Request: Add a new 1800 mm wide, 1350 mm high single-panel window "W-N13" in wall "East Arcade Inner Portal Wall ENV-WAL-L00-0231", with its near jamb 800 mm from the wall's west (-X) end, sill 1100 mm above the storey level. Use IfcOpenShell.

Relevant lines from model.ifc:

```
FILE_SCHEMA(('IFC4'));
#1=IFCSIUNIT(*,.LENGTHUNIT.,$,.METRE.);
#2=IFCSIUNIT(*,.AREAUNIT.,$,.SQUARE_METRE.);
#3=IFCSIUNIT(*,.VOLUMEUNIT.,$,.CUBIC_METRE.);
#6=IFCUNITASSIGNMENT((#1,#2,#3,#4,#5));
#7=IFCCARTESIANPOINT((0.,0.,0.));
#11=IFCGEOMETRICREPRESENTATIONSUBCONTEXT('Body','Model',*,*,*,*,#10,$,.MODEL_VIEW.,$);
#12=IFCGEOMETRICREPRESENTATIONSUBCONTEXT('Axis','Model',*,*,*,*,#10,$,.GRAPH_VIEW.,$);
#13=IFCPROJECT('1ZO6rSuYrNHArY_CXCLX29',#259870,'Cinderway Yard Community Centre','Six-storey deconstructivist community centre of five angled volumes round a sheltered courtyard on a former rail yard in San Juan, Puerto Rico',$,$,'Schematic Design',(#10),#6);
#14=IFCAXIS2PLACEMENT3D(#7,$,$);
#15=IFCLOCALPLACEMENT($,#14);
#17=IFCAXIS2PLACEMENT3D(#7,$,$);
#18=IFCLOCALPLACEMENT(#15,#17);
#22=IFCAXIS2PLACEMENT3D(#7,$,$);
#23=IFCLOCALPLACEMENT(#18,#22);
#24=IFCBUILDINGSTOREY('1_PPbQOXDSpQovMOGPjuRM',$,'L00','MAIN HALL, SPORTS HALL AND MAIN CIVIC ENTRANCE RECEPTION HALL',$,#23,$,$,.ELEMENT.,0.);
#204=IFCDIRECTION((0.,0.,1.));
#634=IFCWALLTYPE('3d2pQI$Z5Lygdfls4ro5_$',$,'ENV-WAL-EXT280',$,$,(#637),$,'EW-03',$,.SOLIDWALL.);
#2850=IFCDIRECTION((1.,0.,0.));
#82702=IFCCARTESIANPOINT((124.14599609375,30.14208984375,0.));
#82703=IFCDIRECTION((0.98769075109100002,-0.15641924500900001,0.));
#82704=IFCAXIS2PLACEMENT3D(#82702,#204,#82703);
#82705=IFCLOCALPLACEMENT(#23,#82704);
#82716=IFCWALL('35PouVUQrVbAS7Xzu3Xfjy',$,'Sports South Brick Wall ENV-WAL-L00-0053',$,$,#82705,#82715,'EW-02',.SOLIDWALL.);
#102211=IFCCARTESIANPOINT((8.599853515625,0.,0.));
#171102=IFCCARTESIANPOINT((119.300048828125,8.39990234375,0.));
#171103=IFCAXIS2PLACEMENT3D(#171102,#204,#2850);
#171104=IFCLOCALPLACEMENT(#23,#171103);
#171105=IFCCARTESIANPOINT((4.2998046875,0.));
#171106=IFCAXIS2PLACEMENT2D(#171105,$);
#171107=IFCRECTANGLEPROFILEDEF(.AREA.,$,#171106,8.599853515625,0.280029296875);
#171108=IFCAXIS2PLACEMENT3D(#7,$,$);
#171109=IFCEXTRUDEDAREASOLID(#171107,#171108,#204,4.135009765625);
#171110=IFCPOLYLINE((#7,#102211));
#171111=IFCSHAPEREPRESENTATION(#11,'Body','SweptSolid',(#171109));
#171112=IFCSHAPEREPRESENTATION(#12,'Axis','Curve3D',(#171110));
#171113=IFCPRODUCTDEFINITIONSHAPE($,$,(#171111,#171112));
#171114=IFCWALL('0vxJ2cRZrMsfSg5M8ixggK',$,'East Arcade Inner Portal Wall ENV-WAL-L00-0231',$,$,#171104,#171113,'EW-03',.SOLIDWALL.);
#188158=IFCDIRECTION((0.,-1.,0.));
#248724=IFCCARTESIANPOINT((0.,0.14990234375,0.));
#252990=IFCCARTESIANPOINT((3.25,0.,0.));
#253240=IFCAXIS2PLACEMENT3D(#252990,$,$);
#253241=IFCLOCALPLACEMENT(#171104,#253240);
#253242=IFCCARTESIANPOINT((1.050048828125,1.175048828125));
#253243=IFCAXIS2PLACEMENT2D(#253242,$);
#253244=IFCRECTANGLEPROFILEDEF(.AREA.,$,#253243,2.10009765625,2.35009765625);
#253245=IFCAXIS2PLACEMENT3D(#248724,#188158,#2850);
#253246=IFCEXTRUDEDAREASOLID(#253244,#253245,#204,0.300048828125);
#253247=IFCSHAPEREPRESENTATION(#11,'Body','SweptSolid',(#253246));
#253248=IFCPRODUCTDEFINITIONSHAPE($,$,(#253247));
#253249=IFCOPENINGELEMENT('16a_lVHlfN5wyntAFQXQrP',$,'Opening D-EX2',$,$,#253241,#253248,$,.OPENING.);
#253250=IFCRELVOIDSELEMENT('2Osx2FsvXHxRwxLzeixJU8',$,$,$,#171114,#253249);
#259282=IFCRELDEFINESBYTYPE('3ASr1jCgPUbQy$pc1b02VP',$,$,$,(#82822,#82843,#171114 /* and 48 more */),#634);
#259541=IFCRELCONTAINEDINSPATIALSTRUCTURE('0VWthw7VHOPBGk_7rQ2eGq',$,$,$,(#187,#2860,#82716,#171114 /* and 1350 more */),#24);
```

```python
import numpy as np
import ifcopenshell
import ifcopenshell.api.feature
import ifcopenshell.api.geometry
import ifcopenshell.api.root
import ifcopenshell.api.spatial
import ifcopenshell.geom
import ifcopenshell.util.element
import ifcopenshell.util.placement
import ifcopenshell.util.representation
import ifcopenshell.util.shape
import ifcopenshell.util.unit

model = ifcopenshell.open("model.ifc")
unit_scale = ifcopenshell.util.unit.calculate_unit_scale(model)
settings = ifcopenshell.geom.settings()


def volume(element):
    """Net volume in cubic metres, openings subtracted."""
    shape = ifcopenshell.geom.create_shape(settings, element)
    return ifcopenshell.util.shape.get_volume(shape.geometry)


wall = model.by_guid("0vxJ2cRZrMsfSg5M8ixggK")
storey = ifcopenshell.util.element.get_container(wall, ifc_class="IfcBuildingStorey")
context = ifcopenshell.util.representation.get_context(model, "Model", "Body", "MODEL_VIEW")
before = volume(wall)

width, height, from_end, sill = 1.8, 1.35, 0.8, 1.1  # metres

# The wall runs along its own X axis, and the end named is its -X end.
wall_shape = ifcopenshell.geom.create_shape(settings, wall)
x, y, z = ifcopenshell.util.shape.get_vertices(wall_shape.geometry).T
start = x.min() + from_end
face, thickness = float(y.min()), float(y.max() - y.min())
wall_matrix = ifcopenshell.util.placement.get_local_placement(wall.ObjectPlacement)
level = ifcopenshell.util.placement.get_local_placement(storey.ObjectPlacement)[2, 3]


def in_wall(x, y):
    """Placement at x, y metres in the wall's axes, at sill height."""
    matrix = wall_matrix.copy()
    matrix[:, 3] = wall_matrix @ np.array([x / unit_scale, y / unit_scale, 0.0, 1.0])
    matrix[2, 3] = level + sill / unit_scale
    return matrix


# Opening: a box that overshoots both wall faces by 50 mm.
opening = ifcopenshell.api.root.create_entity(model, ifc_class="IfcOpeningElement", predefined_type="OPENING")
box = ifcopenshell.api.geometry.add_wall_representation(
    model, context=context, length=width, height=height, thickness=thickness + 0.1
)
ifcopenshell.api.geometry.assign_representation(model, product=opening, representation=box)
ifcopenshell.api.geometry.edit_object_placement(model, product=opening, matrix=in_wall(start, face - 0.05), is_si=False)
ifcopenshell.api.feature.add_feature(model, feature=opening, element=wall)

window = ifcopenshell.api.root.create_entity(model, ifc_class="IfcWindow", name="W-N13", predefined_type="WINDOW")
window.OverallWidth, window.OverallHeight = width / unit_scale, height / unit_scale
window.PartitioningType = "SINGLE_PANEL"
body = ifcopenshell.api.geometry.add_window_representation(
    model,
    context=context,
    overall_width=window.OverallWidth,
    overall_height=window.OverallHeight,
    partition_type="SINGLE_PANEL",
)
ifcopenshell.api.geometry.assign_representation(model, product=window, representation=body)
ifcopenshell.api.spatial.assign_container(model, products=[window], relating_structure=storey)
ifcopenshell.api.feature.add_filling(model, opening=opening, element=window)

# Centre the window in the wall's thickness.
ifcopenshell.api.geometry.edit_object_placement(model, product=window, matrix=in_wall(start, face), is_si=False)
window_shape = ifcopenshell.geom.create_shape(settings, window)
depth = ifcopenshell.util.shape.get_vertices(window_shape.geometry)[:, 1]
offset = face + thickness / 2 - (depth.min() + depth.max()) / 2
ifcopenshell.api.geometry.edit_object_placement(model, product=window, matrix=in_wall(start, offset), is_si=False)

after = volume(wall)

print(f"wall volume {before:.3f} -> {after:.3f} m3")

model.write("model_v2.ifc")
```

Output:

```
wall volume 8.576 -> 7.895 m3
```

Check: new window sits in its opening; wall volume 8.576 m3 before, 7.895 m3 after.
